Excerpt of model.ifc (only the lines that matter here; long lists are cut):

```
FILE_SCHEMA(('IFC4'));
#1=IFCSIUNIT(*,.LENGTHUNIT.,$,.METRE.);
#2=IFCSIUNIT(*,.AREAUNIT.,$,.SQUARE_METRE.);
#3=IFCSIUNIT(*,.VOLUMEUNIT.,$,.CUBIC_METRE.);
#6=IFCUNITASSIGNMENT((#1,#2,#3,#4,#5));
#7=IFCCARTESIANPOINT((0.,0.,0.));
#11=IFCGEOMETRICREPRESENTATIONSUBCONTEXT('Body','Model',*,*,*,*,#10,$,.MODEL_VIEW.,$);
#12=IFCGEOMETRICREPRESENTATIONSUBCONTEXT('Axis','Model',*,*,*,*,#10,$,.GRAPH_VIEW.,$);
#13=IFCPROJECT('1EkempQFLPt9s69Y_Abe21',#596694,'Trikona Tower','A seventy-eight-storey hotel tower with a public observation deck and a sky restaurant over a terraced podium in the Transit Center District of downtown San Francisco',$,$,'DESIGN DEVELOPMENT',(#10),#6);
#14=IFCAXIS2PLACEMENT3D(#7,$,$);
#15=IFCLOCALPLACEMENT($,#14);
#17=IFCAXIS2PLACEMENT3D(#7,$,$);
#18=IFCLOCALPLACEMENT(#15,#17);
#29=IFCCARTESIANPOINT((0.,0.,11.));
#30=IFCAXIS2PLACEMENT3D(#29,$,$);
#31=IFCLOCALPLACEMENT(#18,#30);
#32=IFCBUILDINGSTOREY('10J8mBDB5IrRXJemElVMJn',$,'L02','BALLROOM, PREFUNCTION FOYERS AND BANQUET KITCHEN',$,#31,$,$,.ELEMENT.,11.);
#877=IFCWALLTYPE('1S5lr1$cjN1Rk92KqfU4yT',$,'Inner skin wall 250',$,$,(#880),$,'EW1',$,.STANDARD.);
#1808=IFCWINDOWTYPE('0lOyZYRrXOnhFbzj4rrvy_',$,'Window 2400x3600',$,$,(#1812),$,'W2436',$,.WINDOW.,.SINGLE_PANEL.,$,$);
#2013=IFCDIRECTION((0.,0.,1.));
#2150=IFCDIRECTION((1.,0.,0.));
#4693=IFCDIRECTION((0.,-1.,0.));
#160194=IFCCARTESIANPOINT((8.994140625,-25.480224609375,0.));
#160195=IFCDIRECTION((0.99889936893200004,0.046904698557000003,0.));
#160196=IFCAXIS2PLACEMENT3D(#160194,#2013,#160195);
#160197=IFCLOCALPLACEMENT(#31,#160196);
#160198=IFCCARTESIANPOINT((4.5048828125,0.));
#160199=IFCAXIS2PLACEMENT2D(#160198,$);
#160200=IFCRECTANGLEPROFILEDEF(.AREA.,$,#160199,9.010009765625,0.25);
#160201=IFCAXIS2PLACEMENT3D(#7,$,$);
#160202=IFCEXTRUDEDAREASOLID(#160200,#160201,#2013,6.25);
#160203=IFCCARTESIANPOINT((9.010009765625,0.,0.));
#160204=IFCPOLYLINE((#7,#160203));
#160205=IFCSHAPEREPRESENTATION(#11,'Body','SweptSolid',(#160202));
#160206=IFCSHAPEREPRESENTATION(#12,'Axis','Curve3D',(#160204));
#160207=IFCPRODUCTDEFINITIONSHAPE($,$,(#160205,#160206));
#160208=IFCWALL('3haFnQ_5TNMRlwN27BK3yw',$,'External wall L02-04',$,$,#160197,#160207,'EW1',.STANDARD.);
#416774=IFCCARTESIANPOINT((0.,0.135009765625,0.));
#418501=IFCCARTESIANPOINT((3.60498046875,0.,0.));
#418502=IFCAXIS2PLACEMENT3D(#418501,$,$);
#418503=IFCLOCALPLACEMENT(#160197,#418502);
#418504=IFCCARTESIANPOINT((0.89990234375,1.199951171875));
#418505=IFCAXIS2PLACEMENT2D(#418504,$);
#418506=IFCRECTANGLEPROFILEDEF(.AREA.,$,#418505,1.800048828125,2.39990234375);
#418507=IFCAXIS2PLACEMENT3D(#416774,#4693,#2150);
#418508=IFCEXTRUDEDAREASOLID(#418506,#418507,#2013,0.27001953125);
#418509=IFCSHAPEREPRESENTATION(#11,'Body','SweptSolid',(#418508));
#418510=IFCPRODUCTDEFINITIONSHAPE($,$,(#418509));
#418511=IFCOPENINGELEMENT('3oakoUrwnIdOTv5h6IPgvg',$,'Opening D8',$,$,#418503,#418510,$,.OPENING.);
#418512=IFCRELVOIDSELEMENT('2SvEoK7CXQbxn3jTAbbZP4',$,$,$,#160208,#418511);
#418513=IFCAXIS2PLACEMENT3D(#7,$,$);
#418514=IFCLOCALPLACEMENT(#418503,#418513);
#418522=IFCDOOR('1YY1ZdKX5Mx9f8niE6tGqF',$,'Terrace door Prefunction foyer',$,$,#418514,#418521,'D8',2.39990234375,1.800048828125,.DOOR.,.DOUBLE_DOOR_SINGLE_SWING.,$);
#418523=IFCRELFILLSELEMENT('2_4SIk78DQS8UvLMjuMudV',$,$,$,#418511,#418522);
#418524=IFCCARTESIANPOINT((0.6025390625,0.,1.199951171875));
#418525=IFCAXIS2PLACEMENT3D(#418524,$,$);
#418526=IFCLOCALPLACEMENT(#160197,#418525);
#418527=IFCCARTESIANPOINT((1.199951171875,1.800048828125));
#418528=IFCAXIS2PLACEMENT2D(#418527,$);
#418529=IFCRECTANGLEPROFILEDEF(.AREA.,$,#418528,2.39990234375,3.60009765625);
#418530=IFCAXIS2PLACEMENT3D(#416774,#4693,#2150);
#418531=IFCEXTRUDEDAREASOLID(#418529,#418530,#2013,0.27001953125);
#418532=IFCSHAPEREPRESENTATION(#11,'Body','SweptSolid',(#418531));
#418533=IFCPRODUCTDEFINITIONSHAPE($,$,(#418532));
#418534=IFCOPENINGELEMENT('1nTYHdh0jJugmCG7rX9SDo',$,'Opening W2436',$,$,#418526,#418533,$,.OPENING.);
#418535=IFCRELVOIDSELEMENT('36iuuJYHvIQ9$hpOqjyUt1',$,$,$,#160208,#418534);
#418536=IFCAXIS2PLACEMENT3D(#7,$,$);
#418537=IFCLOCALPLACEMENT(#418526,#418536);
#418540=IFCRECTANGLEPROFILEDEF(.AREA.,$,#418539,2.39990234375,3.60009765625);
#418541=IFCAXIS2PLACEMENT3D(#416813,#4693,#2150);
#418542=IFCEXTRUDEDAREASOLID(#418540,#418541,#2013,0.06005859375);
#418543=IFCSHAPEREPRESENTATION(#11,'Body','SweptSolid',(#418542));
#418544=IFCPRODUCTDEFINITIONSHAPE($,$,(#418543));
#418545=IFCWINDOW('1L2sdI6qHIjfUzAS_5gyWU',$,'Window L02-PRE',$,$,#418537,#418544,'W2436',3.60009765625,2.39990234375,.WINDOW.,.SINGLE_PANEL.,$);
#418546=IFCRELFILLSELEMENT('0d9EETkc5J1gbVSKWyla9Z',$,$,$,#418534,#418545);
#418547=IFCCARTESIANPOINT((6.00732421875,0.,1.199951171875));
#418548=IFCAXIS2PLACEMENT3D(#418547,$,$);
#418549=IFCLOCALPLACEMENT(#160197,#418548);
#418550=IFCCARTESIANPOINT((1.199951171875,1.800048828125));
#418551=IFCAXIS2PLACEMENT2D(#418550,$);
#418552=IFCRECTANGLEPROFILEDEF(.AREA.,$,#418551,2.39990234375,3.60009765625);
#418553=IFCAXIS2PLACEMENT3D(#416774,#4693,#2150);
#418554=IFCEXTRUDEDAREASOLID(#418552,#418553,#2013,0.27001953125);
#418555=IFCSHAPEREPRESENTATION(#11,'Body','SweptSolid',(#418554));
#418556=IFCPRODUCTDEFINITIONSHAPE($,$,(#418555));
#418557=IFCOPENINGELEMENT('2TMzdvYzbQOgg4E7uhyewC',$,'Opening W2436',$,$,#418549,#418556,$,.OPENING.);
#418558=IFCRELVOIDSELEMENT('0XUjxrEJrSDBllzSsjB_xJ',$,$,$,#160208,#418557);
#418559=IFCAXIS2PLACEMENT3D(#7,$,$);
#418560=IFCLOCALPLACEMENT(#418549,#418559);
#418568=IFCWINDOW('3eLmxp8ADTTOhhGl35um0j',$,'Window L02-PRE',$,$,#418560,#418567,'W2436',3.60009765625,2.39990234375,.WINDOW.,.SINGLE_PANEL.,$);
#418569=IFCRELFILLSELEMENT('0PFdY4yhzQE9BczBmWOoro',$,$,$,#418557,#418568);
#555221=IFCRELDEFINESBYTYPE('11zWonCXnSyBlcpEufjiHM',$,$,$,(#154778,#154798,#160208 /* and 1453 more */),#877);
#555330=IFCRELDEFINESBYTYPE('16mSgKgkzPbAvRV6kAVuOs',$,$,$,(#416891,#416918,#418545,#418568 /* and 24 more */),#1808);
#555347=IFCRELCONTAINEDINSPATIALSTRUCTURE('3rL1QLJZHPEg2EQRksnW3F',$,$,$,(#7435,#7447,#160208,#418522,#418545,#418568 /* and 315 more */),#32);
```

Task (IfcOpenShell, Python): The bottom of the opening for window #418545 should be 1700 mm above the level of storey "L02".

```python
import numpy as np
import ifcopenshell
import ifcopenshell.api.geometry
import ifcopenshell.geom
import ifcopenshell.util.element
import ifcopenshell.util.placement
import ifcopenshell.util.shape
import ifcopenshell.util.unit

model = ifcopenshell.open("model.ifc")
unit_scale = ifcopenshell.util.unit.calculate_unit_scale(model)

window = model.by_guid("1L2sdI6qHIjfUzAS_5gyWU")
opening = window.FillsVoids[0].RelatingOpeningElement
storey = ifcopenshell.util.element.get_container(window, ifc_class="IfcBuildingStorey")
level = ifcopenshell.util.placement.get_local_placement(storey.ObjectPlacement)[2, 3]

# The opening's origin need not be at the sill, so measure its lowest point.
shape = ifcopenshell.geom.create_shape(ifcopenshell.geom.settings(), opening)
bottom = ifcopenshell.util.shape.get_shape_bottom_elevation(shape, shape.geometry) / unit_scale
dz = level + 1.7 / unit_scale - bottom

shift = np.array([0.0, 0.0, dz])
# The window is placed relative to its opening, so it follows when the opening moves.
matrix = ifcopenshell.util.placement.get_local_placement(opening.ObjectPlacement)
matrix[:3, 3] += shift
ifcopenshell.api.geometry.edit_object_placement(
    model, product=opening, matrix=matrix, is_si=False, should_transform_children=True
)

print(f"moved by {dz * unit_scale:+.3f} m")

model.write("model_v2.ifc")
```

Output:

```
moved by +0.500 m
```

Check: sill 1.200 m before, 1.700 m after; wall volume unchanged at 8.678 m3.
